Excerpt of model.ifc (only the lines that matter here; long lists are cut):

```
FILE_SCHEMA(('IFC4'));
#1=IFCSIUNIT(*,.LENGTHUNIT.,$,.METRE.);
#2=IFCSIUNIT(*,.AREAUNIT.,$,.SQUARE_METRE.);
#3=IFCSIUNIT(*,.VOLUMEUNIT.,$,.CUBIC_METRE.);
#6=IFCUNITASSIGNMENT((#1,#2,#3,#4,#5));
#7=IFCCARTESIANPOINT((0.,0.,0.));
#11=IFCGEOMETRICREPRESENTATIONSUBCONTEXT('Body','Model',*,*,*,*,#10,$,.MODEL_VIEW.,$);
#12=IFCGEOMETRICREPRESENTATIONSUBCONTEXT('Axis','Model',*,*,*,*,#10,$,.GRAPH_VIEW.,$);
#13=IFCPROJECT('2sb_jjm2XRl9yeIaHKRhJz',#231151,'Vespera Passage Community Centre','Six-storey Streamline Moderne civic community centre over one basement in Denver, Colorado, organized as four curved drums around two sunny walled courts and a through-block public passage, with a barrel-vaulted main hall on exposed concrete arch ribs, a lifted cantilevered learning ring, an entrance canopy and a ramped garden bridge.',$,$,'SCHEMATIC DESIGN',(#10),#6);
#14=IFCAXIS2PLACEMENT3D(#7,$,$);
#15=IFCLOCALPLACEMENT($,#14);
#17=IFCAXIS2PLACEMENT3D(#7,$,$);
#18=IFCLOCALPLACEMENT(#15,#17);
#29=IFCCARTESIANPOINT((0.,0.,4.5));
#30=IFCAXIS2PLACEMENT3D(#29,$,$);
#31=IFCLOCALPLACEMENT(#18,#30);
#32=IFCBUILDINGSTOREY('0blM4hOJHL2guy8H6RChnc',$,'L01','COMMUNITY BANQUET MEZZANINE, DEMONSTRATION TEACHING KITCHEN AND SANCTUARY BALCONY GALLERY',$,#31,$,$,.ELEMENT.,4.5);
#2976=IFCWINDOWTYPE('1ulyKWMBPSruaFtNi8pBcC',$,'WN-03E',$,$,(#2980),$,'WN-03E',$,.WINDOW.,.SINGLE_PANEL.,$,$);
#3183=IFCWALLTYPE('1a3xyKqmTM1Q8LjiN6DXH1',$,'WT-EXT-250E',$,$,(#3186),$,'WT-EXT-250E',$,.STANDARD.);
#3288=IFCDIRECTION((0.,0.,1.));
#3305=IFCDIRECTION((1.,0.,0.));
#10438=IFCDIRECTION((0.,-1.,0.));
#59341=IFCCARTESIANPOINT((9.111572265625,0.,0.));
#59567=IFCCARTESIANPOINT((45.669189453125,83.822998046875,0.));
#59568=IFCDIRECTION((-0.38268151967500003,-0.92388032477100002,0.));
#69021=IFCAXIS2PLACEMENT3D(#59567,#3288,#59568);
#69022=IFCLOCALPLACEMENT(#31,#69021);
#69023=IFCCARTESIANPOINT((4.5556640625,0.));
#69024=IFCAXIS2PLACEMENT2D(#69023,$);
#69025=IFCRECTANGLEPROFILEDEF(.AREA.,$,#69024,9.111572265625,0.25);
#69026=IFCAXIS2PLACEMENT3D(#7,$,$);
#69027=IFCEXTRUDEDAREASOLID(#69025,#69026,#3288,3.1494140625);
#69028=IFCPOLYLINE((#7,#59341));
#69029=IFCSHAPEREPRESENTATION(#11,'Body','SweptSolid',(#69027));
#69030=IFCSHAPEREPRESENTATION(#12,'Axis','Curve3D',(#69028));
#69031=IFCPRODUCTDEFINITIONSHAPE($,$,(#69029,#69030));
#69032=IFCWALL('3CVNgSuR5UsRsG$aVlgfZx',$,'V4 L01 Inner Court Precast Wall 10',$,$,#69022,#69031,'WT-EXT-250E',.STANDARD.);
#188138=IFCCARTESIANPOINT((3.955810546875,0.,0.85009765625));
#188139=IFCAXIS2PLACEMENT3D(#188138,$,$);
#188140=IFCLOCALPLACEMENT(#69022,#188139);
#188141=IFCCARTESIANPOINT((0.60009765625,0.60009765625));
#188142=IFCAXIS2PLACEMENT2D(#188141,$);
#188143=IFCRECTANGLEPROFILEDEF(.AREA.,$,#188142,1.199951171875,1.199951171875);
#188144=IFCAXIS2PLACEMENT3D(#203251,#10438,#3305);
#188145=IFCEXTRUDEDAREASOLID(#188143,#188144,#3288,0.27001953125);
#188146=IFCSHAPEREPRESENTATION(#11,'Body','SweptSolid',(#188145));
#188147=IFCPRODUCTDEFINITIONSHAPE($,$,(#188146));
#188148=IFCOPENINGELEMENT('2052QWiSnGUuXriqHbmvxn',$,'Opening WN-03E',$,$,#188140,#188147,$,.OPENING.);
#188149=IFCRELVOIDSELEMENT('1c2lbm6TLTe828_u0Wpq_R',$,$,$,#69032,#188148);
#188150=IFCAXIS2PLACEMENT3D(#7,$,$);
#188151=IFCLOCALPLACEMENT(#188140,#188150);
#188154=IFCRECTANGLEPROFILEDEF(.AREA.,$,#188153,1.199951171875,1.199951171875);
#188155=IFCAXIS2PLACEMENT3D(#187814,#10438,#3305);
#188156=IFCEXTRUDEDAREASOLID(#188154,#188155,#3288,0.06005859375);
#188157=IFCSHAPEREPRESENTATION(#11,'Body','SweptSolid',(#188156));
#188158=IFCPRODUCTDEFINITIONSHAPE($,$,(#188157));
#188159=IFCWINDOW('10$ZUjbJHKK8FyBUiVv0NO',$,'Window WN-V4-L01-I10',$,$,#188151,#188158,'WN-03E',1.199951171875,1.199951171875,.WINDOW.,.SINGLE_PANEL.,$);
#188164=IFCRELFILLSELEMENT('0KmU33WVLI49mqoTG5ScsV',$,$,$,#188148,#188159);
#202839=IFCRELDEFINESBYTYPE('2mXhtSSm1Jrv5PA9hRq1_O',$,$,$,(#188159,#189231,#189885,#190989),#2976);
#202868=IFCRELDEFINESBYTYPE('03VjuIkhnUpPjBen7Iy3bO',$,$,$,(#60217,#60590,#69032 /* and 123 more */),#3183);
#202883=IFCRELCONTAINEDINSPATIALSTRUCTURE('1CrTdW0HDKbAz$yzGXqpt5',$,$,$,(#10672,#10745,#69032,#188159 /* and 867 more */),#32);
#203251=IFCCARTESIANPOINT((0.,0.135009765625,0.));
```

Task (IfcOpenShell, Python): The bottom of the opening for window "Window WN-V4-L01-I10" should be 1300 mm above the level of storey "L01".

```python
import numpy as np
import ifcopenshell
import ifcopenshell.api.geometry
import ifcopenshell.geom
import ifcopenshell.util.element
import ifcopenshell.util.placement
import ifcopenshell.util.shape
import ifcopenshell.util.unit

model = ifcopenshell.open("model.ifc")
unit_scale = ifcopenshell.util.unit.calculate_unit_scale(model)

window = model.by_id(188159)
opening = window.FillsVoids[0].RelatingOpeningElement
storey = ifcopenshell.util.element.get_container(window, ifc_class="IfcBuildingStorey")
level = ifcopenshell.util.placement.get_local_placement(storey.ObjectPlacement)[2, 3]

# The opening's origin need not be at the sill, so measure its lowest point.
shape = ifcopenshell.geom.create_shape(ifcopenshell.geom.settings(), opening)
bottom = ifcopenshell.util.shape.get_shape_bottom_elevation(shape, shape.geometry) / unit_scale
dz = level + 1.3 / unit_scale - bottom

shift = np.array([0.0, 0.0, dz])
# The window is placed relative to its opening, so it follows when the opening moves.
matrix = ifcopenshell.util.placement.get_local_placement(opening.ObjectPlacement)
matrix[:3, 3] += shift
ifcopenshell.api.geometry.edit_object_placement(
    model, product=opening, matrix=matrix, is_si=False, should_transform_children=True
)

print(f"moved by {dz * unit_scale:+.3f} m")

model.write("model_rev.ifc")
```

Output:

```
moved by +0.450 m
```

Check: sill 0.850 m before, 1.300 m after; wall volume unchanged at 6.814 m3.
